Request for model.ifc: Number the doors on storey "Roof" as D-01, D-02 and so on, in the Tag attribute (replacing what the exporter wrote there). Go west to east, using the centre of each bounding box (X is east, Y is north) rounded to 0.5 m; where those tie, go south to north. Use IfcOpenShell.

First a look at what the model holds.

```python
import ifcopenshell
import ifcopenshell.util.element
import ifcopenshell.util.placement

model = ifcopenshell.open("model.ifc")
print(model.schema)
storey = next(s for s in model.by_type("IfcBuildingStorey") if s.Name == "Roof")
doors = [e for e in ifcopenshell.util.element.get_decomposition(storey) if e.is_a("IfcDoor")]
for e in sorted(doors, key=lambda e: e.id()):
    origin = ifcopenshell.util.placement.get_local_placement(e.ObjectPlacement)[:3, 3]
    print(e.id(), e.Tag, e.Name, origin.round(2) + 0.0, sep=" | ")
```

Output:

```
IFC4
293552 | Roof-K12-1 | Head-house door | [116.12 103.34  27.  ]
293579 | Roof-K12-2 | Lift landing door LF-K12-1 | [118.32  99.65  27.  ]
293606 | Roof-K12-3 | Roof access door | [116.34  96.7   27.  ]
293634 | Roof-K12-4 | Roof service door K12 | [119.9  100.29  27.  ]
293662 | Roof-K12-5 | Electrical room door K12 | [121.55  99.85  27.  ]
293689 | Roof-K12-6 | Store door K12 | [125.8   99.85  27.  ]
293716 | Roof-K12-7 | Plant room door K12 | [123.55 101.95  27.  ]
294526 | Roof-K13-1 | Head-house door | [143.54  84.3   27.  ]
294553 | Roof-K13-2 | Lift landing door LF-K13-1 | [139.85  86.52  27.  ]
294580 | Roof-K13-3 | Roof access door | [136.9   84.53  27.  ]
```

```python
import ifcopenshell
import ifcopenshell.geom
import ifcopenshell.util.element
import ifcopenshell.util.shape

model = ifcopenshell.open("model.ifc")
settings = ifcopenshell.geom.settings()
settings.set("use-world-coords", True)


def centre(element):
    shape = ifcopenshell.geom.create_shape(settings, element)
    return ifcopenshell.util.shape.get_bbox_centroid(shape.geometry)


storey = next(s for s in model.by_type("IfcBuildingStorey") if s.Name == "Roof")
doors = [e for e in ifcopenshell.util.element.get_decomposition(storey) if e.is_a("IfcDoor")]

# Insertion points can sit at a corner or the storey origin, so sort by the geometry (in metres).
centres = {e: centre(e) for e in doors}
doors.sort(key=lambda e: (round(centres[e][0] / 0.5), centres[e][1]))

for i, e in enumerate(doors, start=1):
    number = f"D-{i:02d}"
    e.Tag = number
    print(e.id(), number)

model.write("model_edited.ifc")
```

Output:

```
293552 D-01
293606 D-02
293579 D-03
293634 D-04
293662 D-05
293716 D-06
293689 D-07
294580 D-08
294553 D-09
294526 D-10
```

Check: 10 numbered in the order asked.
